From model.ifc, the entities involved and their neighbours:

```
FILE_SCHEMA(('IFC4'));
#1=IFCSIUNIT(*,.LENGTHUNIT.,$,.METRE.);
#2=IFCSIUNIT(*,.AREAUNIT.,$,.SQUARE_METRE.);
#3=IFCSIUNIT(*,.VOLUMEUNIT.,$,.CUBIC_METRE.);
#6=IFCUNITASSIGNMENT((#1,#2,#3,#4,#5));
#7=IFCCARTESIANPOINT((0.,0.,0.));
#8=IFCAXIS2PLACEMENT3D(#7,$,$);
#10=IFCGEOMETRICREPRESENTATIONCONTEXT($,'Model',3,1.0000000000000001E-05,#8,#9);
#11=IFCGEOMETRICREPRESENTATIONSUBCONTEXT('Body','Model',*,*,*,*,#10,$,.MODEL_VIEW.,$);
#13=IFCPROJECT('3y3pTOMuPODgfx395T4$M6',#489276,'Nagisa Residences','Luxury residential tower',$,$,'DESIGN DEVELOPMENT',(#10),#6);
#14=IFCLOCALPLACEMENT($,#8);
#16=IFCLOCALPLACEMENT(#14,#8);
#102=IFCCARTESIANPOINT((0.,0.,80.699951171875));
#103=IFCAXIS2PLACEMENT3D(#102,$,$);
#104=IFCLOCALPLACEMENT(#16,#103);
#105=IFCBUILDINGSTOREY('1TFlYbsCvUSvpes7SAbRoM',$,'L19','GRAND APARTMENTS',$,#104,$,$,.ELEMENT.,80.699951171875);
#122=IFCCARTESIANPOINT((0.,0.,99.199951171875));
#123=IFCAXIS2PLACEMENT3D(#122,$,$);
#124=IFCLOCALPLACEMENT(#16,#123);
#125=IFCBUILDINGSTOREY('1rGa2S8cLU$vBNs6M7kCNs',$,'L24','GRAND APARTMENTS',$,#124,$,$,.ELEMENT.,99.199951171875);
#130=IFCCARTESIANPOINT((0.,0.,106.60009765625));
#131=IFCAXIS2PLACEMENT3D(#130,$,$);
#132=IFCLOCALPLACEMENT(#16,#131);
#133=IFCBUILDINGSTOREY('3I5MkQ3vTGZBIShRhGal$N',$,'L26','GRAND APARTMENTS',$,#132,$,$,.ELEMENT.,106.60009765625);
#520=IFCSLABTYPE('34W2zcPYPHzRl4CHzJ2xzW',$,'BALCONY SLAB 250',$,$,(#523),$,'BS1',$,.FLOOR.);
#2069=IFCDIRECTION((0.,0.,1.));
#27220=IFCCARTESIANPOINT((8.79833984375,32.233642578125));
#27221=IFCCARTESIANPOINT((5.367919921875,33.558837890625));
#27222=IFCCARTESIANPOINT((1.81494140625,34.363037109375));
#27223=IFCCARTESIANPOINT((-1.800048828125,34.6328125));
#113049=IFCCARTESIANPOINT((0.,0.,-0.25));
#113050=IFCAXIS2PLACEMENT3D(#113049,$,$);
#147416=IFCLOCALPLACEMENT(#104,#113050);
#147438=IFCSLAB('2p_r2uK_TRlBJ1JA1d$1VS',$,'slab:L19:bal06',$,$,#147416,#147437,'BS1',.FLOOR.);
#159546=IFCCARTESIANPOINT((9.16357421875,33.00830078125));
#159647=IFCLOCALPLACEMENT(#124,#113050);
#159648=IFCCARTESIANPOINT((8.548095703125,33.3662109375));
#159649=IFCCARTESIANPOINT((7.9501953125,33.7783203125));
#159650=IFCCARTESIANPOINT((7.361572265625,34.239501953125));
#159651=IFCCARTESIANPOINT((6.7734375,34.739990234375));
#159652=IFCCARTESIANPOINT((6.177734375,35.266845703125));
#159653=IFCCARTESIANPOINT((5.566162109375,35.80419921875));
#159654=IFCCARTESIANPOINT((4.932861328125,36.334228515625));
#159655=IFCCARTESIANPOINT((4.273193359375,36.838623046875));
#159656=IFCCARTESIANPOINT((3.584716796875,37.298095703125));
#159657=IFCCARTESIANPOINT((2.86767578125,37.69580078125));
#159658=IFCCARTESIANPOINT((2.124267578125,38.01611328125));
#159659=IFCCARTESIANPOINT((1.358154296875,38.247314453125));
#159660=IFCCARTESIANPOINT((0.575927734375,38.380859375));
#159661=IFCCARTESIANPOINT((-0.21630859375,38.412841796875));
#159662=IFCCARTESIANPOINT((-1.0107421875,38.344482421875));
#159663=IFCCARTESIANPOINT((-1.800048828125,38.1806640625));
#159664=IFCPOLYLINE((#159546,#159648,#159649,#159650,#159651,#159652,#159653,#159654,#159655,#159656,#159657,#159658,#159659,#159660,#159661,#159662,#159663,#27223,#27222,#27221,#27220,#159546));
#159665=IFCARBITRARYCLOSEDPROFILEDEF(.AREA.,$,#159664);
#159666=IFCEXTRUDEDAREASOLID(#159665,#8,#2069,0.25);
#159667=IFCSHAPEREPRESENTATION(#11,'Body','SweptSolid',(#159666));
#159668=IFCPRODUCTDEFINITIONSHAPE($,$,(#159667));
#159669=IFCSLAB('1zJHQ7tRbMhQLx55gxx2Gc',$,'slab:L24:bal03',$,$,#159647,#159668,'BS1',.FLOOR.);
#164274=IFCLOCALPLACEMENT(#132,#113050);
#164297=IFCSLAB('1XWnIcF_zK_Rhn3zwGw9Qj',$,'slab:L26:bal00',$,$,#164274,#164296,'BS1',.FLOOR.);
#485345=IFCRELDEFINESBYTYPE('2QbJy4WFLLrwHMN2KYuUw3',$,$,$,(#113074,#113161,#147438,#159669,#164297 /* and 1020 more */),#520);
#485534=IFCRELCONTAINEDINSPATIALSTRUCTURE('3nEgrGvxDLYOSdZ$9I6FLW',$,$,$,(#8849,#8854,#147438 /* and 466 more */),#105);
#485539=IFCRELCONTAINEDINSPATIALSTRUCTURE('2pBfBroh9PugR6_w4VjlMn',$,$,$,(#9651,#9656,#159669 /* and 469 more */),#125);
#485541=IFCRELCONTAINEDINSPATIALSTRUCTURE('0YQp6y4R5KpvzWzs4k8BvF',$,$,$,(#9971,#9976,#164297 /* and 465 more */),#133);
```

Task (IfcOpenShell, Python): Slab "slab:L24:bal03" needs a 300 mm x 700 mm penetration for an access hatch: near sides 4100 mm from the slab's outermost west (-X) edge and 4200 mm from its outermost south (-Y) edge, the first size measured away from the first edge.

```python
import numpy as np
import ifcopenshell
import ifcopenshell.api.feature
import ifcopenshell.api.geometry
import ifcopenshell.api.root
import ifcopenshell.geom
import ifcopenshell.util.placement
import ifcopenshell.util.representation
import ifcopenshell.util.shape
import ifcopenshell.util.unit

model = ifcopenshell.open("model.ifc")
unit_scale = ifcopenshell.util.unit.calculate_unit_scale(model)
settings = ifcopenshell.geom.settings()


def volume(element):
    """Net volume in cubic metres, openings subtracted."""
    shape = ifcopenshell.geom.create_shape(settings, element)
    return ifcopenshell.util.shape.get_volume(shape.geometry)


slab = model.by_guid("1zJHQ7tRbMhQLx55gxx2Gc")
before = volume(slab)

# Extent in the slab's own axes, in metres. The edges named are its -X and -Y sides.
slab_shape = ifcopenshell.geom.create_shape(settings, slab)
vertices = ifcopenshell.util.shape.get_vertices(slab_shape.geometry)
x_min, y_min, bottom = vertices.min(axis=0)
top = vertices[:, 2].max()

opening = ifcopenshell.api.root.create_entity(model, ifc_class="IfcOpeningElement", name="Access hatch opening", predefined_type="OPENING")
context = ifcopenshell.util.representation.get_context(model, "Model", "Body", "MODEL_VIEW")
width, depth = 0.3, 0.7
outline = [(0.0, 0.0), (width, 0.0), (width, depth), (0.0, depth), (0.0, 0.0)]
# Overshoot both faces by 50 mm so the cut is clean.
shape = ifcopenshell.api.geometry.add_slab_representation(
    model, context=context, depth=top - bottom + 0.1, polyline=outline
)
ifcopenshell.api.geometry.assign_representation(model, product=opening, representation=shape)

matrix = ifcopenshell.util.placement.get_local_placement(slab.ObjectPlacement)
matrix[:, 3] = matrix @ np.append(np.array([x_min + 4.1, y_min + 4.2, bottom - 0.05]) / unit_scale, 1.0)
ifcopenshell.api.geometry.edit_object_placement(model, product=opening, matrix=matrix, is_si=False)
ifcopenshell.api.feature.add_feature(model, feature=opening, element=slab)

after = volume(slab)

print(f"slab volume {before:.3f} -> {after:.3f} m3")

model.write("model_v2.ifc")
```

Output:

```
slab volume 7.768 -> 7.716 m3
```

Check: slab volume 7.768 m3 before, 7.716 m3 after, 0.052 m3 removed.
